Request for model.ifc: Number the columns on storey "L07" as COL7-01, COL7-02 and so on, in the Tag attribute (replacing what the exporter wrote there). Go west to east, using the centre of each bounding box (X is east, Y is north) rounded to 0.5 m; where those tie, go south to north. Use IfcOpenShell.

First a look at what the model holds.

```python
import ifcopenshell
import ifcopenshell.util.element
import ifcopenshell.util.placement

model = ifcopenshell.open("model.ifc")
print(model.schema)
storey = next(s for s in model.by_type("IfcBuildingStorey") if s.Name == "L07")
columns = [e for e in ifcopenshell.util.element.get_decomposition(storey) if e.is_a("IfcColumn")]
for e in sorted(columns, key=lambda e: e.id()):
    origin = ifcopenshell.util.placement.get_local_placement(e.ObjectPlacement)[:3, 3]
    print(e.id(), e.Tag, e.Name, origin.round(2) + 0.0, sep=" | ")
```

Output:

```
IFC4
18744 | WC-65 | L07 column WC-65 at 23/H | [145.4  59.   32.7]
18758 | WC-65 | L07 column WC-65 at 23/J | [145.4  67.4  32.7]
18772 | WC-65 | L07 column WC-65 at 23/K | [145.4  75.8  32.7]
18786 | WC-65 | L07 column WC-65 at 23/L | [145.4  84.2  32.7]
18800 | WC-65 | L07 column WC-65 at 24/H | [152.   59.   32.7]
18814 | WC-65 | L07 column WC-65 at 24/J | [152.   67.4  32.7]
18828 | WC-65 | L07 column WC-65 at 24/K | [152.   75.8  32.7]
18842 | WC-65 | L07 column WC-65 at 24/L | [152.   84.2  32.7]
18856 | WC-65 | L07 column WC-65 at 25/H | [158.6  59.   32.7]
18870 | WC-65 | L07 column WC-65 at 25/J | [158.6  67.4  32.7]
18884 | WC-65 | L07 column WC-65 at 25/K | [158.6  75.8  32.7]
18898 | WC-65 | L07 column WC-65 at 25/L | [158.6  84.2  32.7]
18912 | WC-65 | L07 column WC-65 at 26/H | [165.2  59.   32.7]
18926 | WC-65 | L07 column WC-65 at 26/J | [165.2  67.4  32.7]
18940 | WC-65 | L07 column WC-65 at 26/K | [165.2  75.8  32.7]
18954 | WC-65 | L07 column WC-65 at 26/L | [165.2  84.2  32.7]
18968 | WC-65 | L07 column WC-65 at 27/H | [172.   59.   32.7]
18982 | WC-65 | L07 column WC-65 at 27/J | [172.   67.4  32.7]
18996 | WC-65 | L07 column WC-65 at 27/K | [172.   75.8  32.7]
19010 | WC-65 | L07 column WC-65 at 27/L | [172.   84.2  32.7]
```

```python
import ifcopenshell
import ifcopenshell.geom
import ifcopenshell.util.element
import ifcopenshell.util.shape

model = ifcopenshell.open("model.ifc")
settings = ifcopenshell.geom.settings()
settings.set("use-world-coords", True)


def centre(element):
    shape = ifcopenshell.geom.create_shape(settings, element)
    return ifcopenshell.util.shape.get_bbox_centroid(shape.geometry)


storey = next(s for s in model.by_type("IfcBuildingStorey") if s.Name == "L07")
columns = [e for e in ifcopenshell.util.element.get_decomposition(storey) if e.is_a("IfcColumn")]

# Insertion points can sit at a corner or the storey origin, so sort by the geometry (in metres).
centres = {e: centre(e) for e in columns}
columns.sort(key=lambda e: (round(centres[e][0] / 0.5), centres[e][1]))

for i, e in enumerate(columns, start=1):
    number = f"COL7-{i:02d}"
    e.Tag = number
    print(e.id(), number)

model.write("model_edited.ifc")
```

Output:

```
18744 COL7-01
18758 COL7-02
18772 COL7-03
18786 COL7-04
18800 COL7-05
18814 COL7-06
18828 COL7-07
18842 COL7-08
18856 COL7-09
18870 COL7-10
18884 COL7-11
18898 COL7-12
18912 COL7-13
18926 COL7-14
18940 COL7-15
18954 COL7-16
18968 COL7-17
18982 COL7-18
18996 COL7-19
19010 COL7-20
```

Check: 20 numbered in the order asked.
